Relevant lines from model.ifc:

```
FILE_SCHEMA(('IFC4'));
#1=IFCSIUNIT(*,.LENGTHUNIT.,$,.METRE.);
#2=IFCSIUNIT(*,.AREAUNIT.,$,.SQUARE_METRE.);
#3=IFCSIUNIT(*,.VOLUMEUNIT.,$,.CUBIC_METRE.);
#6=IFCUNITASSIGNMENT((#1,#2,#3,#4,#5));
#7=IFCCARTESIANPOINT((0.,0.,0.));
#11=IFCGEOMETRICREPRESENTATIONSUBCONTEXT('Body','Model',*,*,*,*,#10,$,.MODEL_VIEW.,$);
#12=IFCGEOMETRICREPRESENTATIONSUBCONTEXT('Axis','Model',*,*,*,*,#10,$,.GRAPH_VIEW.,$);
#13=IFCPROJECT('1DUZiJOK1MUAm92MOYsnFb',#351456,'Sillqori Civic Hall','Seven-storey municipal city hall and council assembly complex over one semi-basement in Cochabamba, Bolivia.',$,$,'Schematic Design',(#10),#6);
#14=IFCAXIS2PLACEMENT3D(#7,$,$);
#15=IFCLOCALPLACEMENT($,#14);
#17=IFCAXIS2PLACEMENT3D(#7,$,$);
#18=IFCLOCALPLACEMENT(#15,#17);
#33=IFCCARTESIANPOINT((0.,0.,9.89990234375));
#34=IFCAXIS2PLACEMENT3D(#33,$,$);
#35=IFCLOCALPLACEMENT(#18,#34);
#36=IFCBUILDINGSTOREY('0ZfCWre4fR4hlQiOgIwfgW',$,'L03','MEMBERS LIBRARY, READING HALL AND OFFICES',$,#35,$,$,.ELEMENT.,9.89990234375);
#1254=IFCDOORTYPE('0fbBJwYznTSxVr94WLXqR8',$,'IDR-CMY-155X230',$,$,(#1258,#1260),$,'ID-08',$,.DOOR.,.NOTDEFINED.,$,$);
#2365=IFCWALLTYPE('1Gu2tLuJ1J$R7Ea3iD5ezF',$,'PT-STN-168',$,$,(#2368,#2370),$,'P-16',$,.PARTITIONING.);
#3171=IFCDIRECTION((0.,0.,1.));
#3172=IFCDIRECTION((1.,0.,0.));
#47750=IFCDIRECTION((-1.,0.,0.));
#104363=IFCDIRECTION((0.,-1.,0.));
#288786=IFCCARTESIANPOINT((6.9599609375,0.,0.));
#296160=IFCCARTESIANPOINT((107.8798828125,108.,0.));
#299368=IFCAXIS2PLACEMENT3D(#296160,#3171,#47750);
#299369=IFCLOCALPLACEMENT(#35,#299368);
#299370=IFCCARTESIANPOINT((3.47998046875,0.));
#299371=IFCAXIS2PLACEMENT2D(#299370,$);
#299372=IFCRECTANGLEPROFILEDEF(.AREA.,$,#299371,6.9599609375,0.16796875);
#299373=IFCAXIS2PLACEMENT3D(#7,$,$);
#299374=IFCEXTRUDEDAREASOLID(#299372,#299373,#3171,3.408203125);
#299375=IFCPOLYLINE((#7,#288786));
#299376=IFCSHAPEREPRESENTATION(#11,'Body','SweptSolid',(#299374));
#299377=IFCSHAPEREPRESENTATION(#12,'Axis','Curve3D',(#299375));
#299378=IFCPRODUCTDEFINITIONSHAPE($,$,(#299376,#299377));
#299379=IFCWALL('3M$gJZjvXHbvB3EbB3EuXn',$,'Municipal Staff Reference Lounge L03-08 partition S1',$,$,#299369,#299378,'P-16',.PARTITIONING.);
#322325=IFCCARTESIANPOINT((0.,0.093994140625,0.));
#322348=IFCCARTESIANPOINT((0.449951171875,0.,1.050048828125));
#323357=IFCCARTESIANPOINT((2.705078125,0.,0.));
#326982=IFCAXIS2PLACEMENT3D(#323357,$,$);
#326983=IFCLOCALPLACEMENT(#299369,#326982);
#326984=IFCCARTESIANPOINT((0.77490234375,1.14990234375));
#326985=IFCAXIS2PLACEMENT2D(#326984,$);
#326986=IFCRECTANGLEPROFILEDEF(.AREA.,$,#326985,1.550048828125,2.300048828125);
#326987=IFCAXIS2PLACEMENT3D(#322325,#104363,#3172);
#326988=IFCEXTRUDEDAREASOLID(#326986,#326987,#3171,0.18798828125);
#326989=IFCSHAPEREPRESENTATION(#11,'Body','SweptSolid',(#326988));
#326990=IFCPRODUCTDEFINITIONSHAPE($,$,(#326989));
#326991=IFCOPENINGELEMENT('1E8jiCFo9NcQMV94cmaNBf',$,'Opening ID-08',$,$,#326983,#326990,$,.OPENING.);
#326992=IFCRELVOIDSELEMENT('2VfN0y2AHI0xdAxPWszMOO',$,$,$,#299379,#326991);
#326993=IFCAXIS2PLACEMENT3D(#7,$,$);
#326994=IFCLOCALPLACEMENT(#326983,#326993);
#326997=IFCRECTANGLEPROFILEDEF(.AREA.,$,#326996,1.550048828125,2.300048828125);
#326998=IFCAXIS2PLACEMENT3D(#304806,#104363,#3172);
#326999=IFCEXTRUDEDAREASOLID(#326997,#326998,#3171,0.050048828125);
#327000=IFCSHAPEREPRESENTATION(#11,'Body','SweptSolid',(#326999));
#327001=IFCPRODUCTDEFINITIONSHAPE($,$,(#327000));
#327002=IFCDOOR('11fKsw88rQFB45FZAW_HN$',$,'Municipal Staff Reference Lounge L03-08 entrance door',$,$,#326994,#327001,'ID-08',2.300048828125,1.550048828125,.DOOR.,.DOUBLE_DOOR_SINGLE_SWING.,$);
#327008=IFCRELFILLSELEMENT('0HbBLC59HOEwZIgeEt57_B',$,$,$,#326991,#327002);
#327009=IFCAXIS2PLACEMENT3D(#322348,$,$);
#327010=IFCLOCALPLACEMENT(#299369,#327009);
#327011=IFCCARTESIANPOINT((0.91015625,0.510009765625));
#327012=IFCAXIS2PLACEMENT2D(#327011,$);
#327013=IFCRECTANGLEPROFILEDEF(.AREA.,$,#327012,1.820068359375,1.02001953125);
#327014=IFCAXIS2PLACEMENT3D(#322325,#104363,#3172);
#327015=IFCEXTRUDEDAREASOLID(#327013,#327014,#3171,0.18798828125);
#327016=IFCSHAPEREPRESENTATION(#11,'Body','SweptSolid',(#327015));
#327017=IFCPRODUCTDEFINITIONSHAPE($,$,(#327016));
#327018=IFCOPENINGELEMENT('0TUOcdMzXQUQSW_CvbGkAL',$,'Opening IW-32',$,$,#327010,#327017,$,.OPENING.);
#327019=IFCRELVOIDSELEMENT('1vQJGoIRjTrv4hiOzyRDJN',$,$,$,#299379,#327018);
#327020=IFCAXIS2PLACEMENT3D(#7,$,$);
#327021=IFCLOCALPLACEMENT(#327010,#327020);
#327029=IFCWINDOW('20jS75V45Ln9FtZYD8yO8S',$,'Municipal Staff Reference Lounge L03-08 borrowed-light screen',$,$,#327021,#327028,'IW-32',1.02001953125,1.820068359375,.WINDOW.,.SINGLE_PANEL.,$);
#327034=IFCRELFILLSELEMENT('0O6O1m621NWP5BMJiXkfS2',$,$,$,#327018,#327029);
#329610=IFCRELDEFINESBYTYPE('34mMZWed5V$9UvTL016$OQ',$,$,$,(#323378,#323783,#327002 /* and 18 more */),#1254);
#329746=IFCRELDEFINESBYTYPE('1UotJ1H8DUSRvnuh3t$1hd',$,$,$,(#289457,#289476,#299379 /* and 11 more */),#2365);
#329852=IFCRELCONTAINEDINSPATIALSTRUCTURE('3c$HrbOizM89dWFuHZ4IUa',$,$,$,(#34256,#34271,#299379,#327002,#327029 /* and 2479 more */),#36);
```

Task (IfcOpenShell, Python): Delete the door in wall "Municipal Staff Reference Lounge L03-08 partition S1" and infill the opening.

```python
import ifcopenshell
import ifcopenshell.api.feature
import ifcopenshell.api.root
import ifcopenshell.geom
import ifcopenshell.util.shape

model = ifcopenshell.open("model.ifc")
settings = ifcopenshell.geom.settings()


def volume(element):
    """Net volume in cubic metres, openings subtracted."""
    shape = ifcopenshell.geom.create_shape(settings, element)
    return ifcopenshell.util.shape.get_volume(shape.geometry)


door = model.by_guid("11fKsw88rQFB45FZAW_HN$")
opening = door.FillsVoids[0].RelatingOpeningElement
wall = opening.VoidsElements[0].RelatingBuildingElement
before = volume(wall)

ifcopenshell.api.root.remove_product(model, product=door)
ifcopenshell.api.feature.remove_feature(model, feature=opening)

after = volume(wall)

print(f"wall volume {before:.3f} -> {after:.3f} m3")

model.write("model_v2.ifc")
```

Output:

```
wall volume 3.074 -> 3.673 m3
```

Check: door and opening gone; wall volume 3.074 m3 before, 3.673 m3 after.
